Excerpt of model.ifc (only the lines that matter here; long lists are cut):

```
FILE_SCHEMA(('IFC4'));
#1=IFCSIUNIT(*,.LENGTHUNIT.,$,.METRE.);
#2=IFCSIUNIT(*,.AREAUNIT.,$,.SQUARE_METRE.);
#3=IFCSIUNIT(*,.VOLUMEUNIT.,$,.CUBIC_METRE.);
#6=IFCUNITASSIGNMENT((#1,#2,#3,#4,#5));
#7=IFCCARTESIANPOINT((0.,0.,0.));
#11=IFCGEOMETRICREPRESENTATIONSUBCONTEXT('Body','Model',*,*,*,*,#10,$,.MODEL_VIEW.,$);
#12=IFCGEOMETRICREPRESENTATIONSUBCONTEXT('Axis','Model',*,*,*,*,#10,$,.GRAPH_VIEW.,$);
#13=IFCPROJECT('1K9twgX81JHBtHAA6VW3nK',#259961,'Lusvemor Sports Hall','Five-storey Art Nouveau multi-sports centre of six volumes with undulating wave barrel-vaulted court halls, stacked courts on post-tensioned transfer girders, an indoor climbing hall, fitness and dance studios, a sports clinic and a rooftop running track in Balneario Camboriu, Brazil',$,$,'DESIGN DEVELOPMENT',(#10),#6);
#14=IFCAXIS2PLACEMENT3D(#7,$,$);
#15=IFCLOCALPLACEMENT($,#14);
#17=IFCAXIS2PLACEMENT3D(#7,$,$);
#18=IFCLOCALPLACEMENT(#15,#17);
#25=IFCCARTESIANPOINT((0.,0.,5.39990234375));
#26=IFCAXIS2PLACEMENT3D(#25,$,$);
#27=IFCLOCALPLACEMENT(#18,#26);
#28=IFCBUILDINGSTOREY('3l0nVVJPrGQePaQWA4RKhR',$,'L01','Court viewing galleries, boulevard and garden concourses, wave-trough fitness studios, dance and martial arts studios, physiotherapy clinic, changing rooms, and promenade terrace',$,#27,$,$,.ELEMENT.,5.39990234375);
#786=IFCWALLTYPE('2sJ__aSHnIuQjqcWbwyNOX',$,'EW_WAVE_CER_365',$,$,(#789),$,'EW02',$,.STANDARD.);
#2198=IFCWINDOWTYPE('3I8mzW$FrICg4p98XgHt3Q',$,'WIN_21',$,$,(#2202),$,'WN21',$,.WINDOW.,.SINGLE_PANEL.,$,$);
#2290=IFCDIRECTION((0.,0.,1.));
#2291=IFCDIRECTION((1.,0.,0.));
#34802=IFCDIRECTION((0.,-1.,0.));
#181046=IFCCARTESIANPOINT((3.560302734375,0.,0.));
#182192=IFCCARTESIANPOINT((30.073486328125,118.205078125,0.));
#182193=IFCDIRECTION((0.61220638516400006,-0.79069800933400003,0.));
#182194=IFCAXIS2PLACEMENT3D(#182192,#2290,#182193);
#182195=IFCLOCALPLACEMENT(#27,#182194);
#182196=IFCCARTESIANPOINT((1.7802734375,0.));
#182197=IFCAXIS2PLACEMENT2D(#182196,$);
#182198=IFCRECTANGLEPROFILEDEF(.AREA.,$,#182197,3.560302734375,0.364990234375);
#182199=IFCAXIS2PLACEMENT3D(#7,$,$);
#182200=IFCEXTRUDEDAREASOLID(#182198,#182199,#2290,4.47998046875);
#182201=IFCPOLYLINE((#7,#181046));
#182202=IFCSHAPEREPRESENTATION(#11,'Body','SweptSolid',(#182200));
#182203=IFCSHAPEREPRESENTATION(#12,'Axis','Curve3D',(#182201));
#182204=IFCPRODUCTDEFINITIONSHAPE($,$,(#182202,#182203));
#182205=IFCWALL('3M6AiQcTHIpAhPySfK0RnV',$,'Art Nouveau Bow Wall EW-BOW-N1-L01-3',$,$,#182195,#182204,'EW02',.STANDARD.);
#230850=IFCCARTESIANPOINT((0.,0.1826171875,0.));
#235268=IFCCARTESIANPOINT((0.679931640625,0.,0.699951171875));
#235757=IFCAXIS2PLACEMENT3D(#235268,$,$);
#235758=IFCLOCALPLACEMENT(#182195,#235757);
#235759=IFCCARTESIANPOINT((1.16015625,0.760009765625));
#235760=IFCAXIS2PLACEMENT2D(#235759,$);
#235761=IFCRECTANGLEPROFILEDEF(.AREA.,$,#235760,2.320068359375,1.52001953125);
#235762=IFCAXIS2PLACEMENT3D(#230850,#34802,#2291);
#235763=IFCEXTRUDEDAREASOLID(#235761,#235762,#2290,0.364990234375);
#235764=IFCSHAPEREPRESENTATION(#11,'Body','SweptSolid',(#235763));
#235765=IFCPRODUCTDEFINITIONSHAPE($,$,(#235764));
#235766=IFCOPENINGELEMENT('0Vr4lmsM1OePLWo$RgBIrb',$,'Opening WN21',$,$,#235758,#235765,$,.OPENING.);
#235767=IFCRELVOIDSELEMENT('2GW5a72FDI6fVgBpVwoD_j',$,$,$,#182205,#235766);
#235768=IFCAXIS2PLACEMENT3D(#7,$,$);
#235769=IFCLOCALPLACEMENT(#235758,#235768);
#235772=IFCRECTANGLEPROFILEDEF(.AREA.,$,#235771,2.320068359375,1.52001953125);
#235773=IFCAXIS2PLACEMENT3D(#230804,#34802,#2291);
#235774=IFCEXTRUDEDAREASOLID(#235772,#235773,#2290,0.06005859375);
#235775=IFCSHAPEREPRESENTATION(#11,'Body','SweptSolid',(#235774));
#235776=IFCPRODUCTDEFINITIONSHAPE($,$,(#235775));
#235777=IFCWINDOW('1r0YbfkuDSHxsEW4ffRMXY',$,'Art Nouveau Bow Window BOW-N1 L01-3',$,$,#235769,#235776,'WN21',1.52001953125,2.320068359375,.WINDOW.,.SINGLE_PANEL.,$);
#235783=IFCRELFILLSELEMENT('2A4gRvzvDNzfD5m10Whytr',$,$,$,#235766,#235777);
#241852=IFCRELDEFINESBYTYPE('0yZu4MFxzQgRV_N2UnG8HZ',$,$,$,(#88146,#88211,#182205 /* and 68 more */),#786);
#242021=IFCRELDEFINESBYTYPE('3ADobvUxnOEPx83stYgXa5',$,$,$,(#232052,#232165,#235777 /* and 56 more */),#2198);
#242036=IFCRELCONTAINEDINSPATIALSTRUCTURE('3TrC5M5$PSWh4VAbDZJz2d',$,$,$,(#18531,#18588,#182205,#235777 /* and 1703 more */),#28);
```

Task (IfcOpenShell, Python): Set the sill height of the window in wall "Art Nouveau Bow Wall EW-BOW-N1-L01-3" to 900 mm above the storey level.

```python
import numpy as np
import ifcopenshell
import ifcopenshell.api.geometry
import ifcopenshell.geom
import ifcopenshell.util.element
import ifcopenshell.util.placement
import ifcopenshell.util.shape
import ifcopenshell.util.unit

model = ifcopenshell.open("model.ifc")
unit_scale = ifcopenshell.util.unit.calculate_unit_scale(model)

window = model.by_guid("1r0YbfkuDSHxsEW4ffRMXY")
opening = window.FillsVoids[0].RelatingOpeningElement
storey = ifcopenshell.util.element.get_container(window, ifc_class="IfcBuildingStorey")
level = ifcopenshell.util.placement.get_local_placement(storey.ObjectPlacement)[2, 3]

# The opening's origin need not be at the sill, so measure its lowest point.
shape = ifcopenshell.geom.create_shape(ifcopenshell.geom.settings(), opening)
bottom = ifcopenshell.util.shape.get_shape_bottom_elevation(shape, shape.geometry) / unit_scale
dz = level + 0.9 / unit_scale - bottom

shift = np.array([0.0, 0.0, dz])
# The window is placed relative to its opening, so it follows when the opening moves.
matrix = ifcopenshell.util.placement.get_local_placement(opening.ObjectPlacement)
matrix[:3, 3] += shift
ifcopenshell.api.geometry.edit_object_placement(
    model, product=opening, matrix=matrix, is_si=False, should_transform_children=True
)

print(f"moved by {dz * unit_scale:+.3f} m")

model.write("model_v2.ifc")
```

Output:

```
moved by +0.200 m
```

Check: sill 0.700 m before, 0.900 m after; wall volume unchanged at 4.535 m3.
